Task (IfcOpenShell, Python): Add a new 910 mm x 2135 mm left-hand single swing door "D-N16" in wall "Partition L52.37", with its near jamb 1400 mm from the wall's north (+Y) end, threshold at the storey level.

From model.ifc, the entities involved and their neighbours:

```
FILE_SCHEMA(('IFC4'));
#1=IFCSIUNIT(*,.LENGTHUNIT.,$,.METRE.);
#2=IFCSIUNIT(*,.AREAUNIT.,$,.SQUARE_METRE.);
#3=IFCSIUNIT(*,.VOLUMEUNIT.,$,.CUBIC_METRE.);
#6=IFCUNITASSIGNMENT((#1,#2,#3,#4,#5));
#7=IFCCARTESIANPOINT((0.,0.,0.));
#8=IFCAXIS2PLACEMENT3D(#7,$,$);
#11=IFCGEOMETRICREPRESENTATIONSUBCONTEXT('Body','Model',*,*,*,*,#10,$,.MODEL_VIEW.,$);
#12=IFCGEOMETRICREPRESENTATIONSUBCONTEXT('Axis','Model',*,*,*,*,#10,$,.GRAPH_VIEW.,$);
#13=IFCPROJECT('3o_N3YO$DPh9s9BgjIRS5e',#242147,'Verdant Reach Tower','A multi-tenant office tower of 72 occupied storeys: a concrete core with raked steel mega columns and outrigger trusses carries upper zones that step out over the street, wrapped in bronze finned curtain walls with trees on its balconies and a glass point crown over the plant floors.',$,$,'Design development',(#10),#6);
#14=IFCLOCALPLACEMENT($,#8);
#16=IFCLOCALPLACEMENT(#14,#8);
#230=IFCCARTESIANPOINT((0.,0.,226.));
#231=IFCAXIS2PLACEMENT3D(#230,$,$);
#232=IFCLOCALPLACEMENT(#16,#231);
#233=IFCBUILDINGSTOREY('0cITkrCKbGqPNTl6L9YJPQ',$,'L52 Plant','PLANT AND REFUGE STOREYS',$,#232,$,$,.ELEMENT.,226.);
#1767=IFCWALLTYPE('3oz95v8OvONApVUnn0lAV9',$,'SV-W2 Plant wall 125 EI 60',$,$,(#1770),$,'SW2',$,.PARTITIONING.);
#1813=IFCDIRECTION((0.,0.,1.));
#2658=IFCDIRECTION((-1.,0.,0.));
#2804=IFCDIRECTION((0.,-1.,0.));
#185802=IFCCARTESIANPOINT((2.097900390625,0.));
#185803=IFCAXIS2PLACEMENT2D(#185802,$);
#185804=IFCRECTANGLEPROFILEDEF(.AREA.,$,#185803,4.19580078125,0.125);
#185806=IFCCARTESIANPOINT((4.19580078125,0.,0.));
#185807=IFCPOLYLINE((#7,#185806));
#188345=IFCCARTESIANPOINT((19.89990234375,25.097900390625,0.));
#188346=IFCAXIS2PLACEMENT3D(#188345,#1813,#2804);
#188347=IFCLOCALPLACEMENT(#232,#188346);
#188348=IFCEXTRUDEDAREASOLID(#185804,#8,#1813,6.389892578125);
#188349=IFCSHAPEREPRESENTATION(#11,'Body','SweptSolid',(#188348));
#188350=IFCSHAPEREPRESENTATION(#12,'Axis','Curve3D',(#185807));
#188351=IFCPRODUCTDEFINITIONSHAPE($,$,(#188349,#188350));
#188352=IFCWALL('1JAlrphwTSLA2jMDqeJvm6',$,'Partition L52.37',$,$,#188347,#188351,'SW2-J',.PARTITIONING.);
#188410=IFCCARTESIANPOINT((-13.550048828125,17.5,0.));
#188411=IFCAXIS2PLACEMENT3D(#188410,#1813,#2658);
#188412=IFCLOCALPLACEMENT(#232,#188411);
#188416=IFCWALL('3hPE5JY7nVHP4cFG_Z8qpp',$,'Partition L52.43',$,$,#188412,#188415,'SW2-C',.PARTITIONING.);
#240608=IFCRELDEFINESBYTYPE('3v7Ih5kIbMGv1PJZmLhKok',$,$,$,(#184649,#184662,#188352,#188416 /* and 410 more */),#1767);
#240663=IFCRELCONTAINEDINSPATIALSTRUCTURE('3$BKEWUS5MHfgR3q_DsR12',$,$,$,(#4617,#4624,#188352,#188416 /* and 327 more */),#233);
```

```python
import numpy as np
import ifcopenshell
import ifcopenshell.api.feature
import ifcopenshell.api.geometry
import ifcopenshell.api.root
import ifcopenshell.api.spatial
import ifcopenshell.geom
import ifcopenshell.util.element
import ifcopenshell.util.placement
import ifcopenshell.util.representation
import ifcopenshell.util.shape
import ifcopenshell.util.unit

model = ifcopenshell.open("model.ifc")
unit_scale = ifcopenshell.util.unit.calculate_unit_scale(model)
settings = ifcopenshell.geom.settings()


def volume(element):
    """Net volume in cubic metres, openings subtracted."""
    shape = ifcopenshell.geom.create_shape(settings, element)
    return ifcopenshell.util.shape.get_volume(shape.geometry)


wall = model.by_guid("1JAlrphwTSLA2jMDqeJvm6")
storey = ifcopenshell.util.element.get_container(wall, ifc_class="IfcBuildingStorey")
context = ifcopenshell.util.representation.get_context(model, "Model", "Body", "MODEL_VIEW")
before = volume(wall)

width, height, from_end, sill = 0.91, 2.135, 1.4, 0.0  # metres

# The wall runs along its own X axis, and the end named is its -X end.
wall_shape = ifcopenshell.geom.create_shape(settings, wall)
x, y, z = ifcopenshell.util.shape.get_vertices(wall_shape.geometry).T
start = x.min() + from_end
face, thickness = float(y.min()), float(y.max() - y.min())
wall_matrix = ifcopenshell.util.placement.get_local_placement(wall.ObjectPlacement)
level = ifcopenshell.util.placement.get_local_placement(storey.ObjectPlacement)[2, 3]


def in_wall(x, y):
    """Placement at x, y metres in the wall's axes, at sill height."""
    matrix = wall_matrix.copy()
    matrix[:, 3] = wall_matrix @ np.array([x / unit_scale, y / unit_scale, 0.0, 1.0])
    matrix[2, 3] = level + sill / unit_scale
    return matrix


# Opening: a box that overshoots both wall faces by 50 mm.
opening = ifcopenshell.api.root.create_entity(model, ifc_class="IfcOpeningElement", predefined_type="OPENING")
box = ifcopenshell.api.geometry.add_wall_representation(
    model, context=context, length=width, height=height, thickness=thickness + 0.1
)
ifcopenshell.api.geometry.assign_representation(model, product=opening, representation=box)
ifcopenshell.api.geometry.edit_object_placement(model, product=opening, matrix=in_wall(start, face - 0.05), is_si=False)
ifcopenshell.api.feature.add_feature(model, feature=opening, element=wall)

door = ifcopenshell.api.root.create_entity(model, ifc_class="IfcDoor", name="D-N16", predefined_type="DOOR")
door.OverallWidth, door.OverallHeight = width / unit_scale, height / unit_scale
door.OperationType = "SINGLE_SWING_LEFT"
body = ifcopenshell.api.geometry.add_door_representation(
    model,
    context=context,
    overall_width=door.OverallWidth,
    overall_height=door.OverallHeight,
    operation_type="SINGLE_SWING_LEFT",
    lining_properties={"LiningDepth": thickness / unit_scale, "ThresholdDepth": thickness / unit_scale},
)
ifcopenshell.api.geometry.assign_representation(model, product=door, representation=body)
ifcopenshell.api.spatial.assign_container(model, products=[door], relating_structure=storey)
ifcopenshell.api.feature.add_filling(model, opening=opening, element=door)

# The lining spans the wall, so the door starts at the wall face.
ifcopenshell.api.geometry.edit_object_placement(model, product=door, matrix=in_wall(start, face), is_si=False)

after = volume(wall)

print(f"wall volume {before:.3f} -> {after:.3f} m3")

model.write("model_edited.ifc")
```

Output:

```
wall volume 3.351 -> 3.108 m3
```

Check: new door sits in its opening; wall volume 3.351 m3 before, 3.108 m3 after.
